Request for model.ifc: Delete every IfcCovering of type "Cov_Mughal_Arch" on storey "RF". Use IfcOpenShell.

First a look at what the model holds.

```python
import ifcopenshell
import ifcopenshell.util.element

model = ifcopenshell.open("model.ifc")
print(model.schema)
storey = next(s for s in model.by_type("IfcBuildingStorey") if s.Name == "RF")
coverings = [e for e in ifcopenshell.util.element.get_decomposition(storey) if e.is_a("IfcCovering")]
seen = {}
for e in coverings:
    element_type = ifcopenshell.util.element.get_type(e)
    name = element_type.Name if element_type not in (None, e) else None
    seen[name] = seen.get(name, 0) + 1
for name, count in sorted(seen.items(), key=str):
    print(count, "x", name)
```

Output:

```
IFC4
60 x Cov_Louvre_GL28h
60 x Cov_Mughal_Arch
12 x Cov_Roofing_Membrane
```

```python
import ifcopenshell
import ifcopenshell.api.root
import ifcopenshell.util.element

model = ifcopenshell.open("model.ifc")

storey = next(s for s in model.by_type("IfcBuildingStorey") if s.Name == "RF")
coverings = [e for e in ifcopenshell.util.element.get_decomposition(storey) if e.is_a("IfcCovering")]
targets = [e for e in coverings if (t := ifcopenshell.util.element.get_type(e)) not in (None, e) and t.Name == "Cov_Mughal_Arch"]

for e in targets:
    ifcopenshell.api.root.remove_product(model, product=e)
print(len(targets), "removed")

model.write("model_v2.ifc")
```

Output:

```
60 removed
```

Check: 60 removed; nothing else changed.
